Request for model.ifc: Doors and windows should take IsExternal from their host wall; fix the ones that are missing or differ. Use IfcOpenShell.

First a look at what the model holds.

```python
import ifcopenshell
import ifcopenshell.util.element

model = ifcopenshell.open("model.ifc")
print(model.schema)
seen = {}
for e in model.by_type("IfcDoor") + model.by_type("IfcWindow"):
    if not e.FillsVoids:
        continue
    host = e.FillsVoids[0].RelatingOpeningElement.VoidsElements[0].RelatingBuildingElement
    own = ifcopenshell.util.element.get_pset(e, f"Pset_{e.is_a()[3:].removesuffix('StandardCase')}Common", "IsExternal")
    wall = ifcopenshell.util.element.get_pset(host, "Pset_WallCommon", "IsExternal")
    seen[e.is_a(), own, wall] = seen.get((e.is_a(), own, wall), 0) + 1
for (cls, own, wall), count in sorted(seen.items(), key=str):
    print(count, cls, "IsExternal:", own, "| host wall:", wall)
```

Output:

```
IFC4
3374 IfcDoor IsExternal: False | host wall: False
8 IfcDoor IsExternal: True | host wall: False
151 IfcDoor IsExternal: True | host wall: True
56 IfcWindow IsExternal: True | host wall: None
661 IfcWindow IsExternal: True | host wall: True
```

```python
import ifcopenshell
import ifcopenshell.api.pset
import ifcopenshell.util.element

model = ifcopenshell.open("model.ifc")

count = 0
for ifc_class, pset_name in (("IfcDoor", "Pset_DoorCommon"), ("IfcWindow", "Pset_WindowCommon")):
    for e in model.by_type(ifc_class):
        if not e.FillsVoids:
            continue
        host = e.FillsVoids[0].RelatingOpeningElement.VoidsElements[0].RelatingBuildingElement
        external = ifcopenshell.util.element.get_pset(host, "Pset_WallCommon", "IsExternal")
        if external is None or ifcopenshell.util.element.get_pset(e, pset_name, "IsExternal") == external:
            continue
        pset = ifcopenshell.api.pset.add_pset(model, product=e, name=pset_name)
        ifcopenshell.api.pset.edit_pset(model, pset=pset, properties={"IsExternal": external})
        count += 1

print(count, "updated")

model.write("model_updated.ifc")
```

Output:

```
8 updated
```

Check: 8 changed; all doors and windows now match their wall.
